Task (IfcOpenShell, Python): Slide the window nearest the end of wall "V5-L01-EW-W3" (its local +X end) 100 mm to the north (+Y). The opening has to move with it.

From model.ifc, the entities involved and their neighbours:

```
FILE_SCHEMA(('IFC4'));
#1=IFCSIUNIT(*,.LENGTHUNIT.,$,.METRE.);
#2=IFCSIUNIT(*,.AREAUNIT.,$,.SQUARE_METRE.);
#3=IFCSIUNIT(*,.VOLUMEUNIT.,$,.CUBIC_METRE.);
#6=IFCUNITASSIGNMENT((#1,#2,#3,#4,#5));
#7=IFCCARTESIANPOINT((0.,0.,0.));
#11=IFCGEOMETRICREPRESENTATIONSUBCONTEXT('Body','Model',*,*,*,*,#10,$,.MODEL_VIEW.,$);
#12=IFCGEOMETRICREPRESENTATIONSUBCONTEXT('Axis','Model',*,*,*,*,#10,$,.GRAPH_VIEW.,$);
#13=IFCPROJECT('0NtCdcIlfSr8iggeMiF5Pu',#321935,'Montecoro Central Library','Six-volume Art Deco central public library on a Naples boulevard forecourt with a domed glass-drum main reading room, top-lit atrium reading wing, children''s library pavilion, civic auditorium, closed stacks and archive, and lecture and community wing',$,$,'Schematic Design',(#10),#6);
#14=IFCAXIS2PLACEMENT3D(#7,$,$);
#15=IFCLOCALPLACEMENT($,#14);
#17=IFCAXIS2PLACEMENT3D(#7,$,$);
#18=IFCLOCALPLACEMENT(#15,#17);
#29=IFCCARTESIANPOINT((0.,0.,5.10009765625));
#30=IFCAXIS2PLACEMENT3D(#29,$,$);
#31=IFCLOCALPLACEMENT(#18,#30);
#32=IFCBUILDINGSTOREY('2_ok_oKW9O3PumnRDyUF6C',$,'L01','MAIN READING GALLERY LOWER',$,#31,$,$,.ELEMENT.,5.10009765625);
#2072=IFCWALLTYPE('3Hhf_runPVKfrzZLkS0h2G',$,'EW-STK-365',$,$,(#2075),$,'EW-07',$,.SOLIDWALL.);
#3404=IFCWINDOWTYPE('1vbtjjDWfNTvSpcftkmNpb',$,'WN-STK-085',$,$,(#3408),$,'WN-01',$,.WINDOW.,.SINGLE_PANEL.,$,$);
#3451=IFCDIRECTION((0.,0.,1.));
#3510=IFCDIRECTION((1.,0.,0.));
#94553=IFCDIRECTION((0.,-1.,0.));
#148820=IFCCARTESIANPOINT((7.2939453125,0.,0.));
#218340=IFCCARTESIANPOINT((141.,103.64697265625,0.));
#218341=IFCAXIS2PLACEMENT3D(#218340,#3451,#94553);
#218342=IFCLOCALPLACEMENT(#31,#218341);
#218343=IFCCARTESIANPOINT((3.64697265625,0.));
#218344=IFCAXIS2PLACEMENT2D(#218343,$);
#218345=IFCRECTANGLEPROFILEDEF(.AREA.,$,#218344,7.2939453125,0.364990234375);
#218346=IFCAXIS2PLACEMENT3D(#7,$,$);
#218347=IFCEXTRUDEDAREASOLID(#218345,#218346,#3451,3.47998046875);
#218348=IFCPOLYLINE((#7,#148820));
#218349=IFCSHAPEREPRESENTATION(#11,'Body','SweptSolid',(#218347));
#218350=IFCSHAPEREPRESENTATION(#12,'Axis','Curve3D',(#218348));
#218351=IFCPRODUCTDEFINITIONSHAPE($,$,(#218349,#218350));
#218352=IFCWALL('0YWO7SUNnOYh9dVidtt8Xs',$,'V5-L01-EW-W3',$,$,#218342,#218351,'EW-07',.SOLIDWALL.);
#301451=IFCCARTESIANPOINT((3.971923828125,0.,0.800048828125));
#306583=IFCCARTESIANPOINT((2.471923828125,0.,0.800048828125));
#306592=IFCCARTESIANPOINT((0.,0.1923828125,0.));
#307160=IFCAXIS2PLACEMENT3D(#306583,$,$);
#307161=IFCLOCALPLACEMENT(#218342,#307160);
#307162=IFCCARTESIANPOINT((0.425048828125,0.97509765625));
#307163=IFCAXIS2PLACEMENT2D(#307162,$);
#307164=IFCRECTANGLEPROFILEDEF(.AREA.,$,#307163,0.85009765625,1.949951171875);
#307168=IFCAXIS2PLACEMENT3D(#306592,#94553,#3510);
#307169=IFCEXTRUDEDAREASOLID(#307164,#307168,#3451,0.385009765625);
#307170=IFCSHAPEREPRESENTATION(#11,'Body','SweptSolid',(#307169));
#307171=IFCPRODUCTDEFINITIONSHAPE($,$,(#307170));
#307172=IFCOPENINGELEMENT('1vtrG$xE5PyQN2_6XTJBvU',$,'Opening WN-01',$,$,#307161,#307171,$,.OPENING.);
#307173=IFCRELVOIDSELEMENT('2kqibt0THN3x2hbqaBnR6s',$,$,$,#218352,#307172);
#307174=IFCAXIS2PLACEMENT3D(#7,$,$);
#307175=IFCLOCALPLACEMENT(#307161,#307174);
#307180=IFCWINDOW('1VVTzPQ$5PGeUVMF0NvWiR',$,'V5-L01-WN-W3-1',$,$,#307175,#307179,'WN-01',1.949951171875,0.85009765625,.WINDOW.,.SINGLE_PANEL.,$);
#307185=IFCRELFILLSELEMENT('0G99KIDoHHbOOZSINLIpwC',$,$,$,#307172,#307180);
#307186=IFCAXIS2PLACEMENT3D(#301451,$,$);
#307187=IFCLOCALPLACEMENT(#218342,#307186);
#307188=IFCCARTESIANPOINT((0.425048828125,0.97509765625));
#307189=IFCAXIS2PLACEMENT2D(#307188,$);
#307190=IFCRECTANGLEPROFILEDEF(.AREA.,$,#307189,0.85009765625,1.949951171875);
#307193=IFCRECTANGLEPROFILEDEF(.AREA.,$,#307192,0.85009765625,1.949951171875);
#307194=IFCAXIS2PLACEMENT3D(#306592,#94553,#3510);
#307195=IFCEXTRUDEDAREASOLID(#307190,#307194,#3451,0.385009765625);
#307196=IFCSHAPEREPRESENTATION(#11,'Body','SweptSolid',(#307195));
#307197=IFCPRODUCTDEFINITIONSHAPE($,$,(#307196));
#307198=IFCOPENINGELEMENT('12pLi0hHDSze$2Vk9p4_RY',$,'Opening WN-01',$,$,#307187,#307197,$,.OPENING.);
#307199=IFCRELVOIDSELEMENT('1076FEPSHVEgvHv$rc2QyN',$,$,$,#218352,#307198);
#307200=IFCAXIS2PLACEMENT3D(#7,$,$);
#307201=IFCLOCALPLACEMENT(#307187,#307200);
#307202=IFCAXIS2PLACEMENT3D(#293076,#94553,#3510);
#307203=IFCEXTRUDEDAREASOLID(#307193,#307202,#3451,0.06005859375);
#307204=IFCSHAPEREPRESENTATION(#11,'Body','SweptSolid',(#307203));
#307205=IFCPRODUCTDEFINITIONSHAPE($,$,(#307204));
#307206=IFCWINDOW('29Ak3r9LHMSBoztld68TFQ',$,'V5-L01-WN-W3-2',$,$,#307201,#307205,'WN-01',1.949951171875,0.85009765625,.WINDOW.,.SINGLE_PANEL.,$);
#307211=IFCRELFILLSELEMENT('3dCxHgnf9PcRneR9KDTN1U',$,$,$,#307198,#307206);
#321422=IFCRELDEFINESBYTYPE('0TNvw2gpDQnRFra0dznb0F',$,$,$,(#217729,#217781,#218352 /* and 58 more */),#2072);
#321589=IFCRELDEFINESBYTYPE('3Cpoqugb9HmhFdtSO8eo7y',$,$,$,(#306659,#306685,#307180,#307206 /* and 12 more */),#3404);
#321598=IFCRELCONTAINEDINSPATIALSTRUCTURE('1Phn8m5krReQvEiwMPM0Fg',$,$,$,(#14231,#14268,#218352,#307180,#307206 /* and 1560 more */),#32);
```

```python
import ifcopenshell
import ifcopenshell.api.geometry
import ifcopenshell.util.placement

model = ifcopenshell.open("model.ifc")

window = model.by_id(307206)
opening = window.FillsVoids[0].RelatingOpeningElement
wall = opening.VoidsElements[0].RelatingBuildingElement

wall_matrix = ifcopenshell.util.placement.get_local_placement(wall.ObjectPlacement)
shift = wall_matrix[:3, 0] * -0.1
before = ifcopenshell.util.placement.get_local_placement(window.ObjectPlacement)[:3, 3].copy()

# The window is placed relative to its opening, so it follows when the opening moves.
matrix = ifcopenshell.util.placement.get_local_placement(opening.ObjectPlacement)
matrix[:3, 3] += shift
ifcopenshell.api.geometry.edit_object_placement(
    model, product=opening, matrix=matrix, is_si=False, should_transform_children=True
)

after = ifcopenshell.util.placement.get_local_placement(window.ObjectPlacement)[:3, 3]
print("window moved by", (after - before).round(3) + 0.0)

model.write("model_v2.ifc")
```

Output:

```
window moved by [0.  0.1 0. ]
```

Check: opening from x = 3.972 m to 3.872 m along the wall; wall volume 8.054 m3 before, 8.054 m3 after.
